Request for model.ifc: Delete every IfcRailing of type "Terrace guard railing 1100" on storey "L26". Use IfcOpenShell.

First a look at what the model holds.

```python
import ifcopenshell
import ifcopenshell.util.element

model = ifcopenshell.open("model.ifc")
print(model.schema)
storey = next(s for s in model.by_type("IfcBuildingStorey") if s.Name == "L26")
railings = [e for e in ifcopenshell.util.element.get_decomposition(storey) if e.is_a("IfcRailing")]
seen = {}
for e in railings:
    element_type = ifcopenshell.util.element.get_type(e)
    name = element_type.Name if element_type not in (None, e) else None
    seen[name] = seen.get(name, 0) + 1
for name, count in sorted(seen.items(), key=str):
    print(count, "x", name)
```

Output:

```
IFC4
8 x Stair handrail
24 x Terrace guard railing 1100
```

```python
import ifcopenshell
import ifcopenshell.api.root
import ifcopenshell.util.element

model = ifcopenshell.open("model.ifc")

storey = next(s for s in model.by_type("IfcBuildingStorey") if s.Name == "L26")
railings = [e for e in ifcopenshell.util.element.get_decomposition(storey) if e.is_a("IfcRailing")]
targets = [e for e in railings if (t := ifcopenshell.util.element.get_type(e)) not in (None, e) and t.Name == "Terrace guard railing 1100"]

for e in targets:
    ifcopenshell.api.root.remove_product(model, product=e)
print(len(targets), "removed")

model.write("model_edited.ifc")
```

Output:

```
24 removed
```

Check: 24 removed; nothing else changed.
